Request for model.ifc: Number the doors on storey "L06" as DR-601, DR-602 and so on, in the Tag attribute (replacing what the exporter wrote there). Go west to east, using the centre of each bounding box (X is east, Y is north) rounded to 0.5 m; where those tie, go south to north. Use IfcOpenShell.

First a look at what the model holds.

```python
import ifcopenshell
import ifcopenshell.util.element
import ifcopenshell.util.placement

model = ifcopenshell.open("model.ifc")
print(model.schema)
storey = next(s for s in model.by_type("IfcBuildingStorey") if s.Name == "L06")
doors = [e for e in ifcopenshell.util.element.get_decomposition(storey) if e.is_a("IfcDoor")]
for e in sorted(doors, key=lambda e: e.id()):
    origin = ifcopenshell.util.placement.get_local_placement(e.ObjectPlacement)[:3, 3]
    print(e.id(), e.Tag, e.Name, origin.round(2) + 0.0, sep=" | ")
```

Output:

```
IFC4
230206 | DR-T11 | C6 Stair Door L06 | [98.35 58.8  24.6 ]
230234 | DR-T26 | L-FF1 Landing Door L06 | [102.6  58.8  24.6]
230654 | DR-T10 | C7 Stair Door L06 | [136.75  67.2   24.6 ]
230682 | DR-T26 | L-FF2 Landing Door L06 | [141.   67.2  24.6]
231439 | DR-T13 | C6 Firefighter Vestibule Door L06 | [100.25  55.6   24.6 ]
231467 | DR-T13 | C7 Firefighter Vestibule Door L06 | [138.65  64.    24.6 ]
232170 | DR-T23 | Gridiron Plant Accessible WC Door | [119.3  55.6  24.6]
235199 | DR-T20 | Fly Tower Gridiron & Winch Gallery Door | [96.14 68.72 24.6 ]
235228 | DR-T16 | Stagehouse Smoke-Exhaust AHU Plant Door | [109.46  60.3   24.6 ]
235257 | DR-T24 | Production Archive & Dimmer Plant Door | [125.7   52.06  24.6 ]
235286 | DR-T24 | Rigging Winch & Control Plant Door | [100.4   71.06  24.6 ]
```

```python
import ifcopenshell
import ifcopenshell.geom
import ifcopenshell.util.element
import ifcopenshell.util.shape

model = ifcopenshell.open("model.ifc")
settings = ifcopenshell.geom.settings()
settings.set("use-world-coords", True)


def centre(element):
    shape = ifcopenshell.geom.create_shape(settings, element)
    return ifcopenshell.util.shape.get_bbox_centroid(shape.geometry)


storey = next(s for s in model.by_type("IfcBuildingStorey") if s.Name == "L06")
doors = [e for e in ifcopenshell.util.element.get_decomposition(storey) if e.is_a("IfcDoor")]

# Insertion points can sit at a corner or the storey origin, so sort by the geometry (in metres).
centres = {e: centre(e) for e in doors}
doors.sort(key=lambda e: (round(centres[e][0] / 0.5), centres[e][1]))

for i, e in enumerate(doors, start=1):
    number = f"DR-6{i:02d}"
    e.Tag = number
    print(e.id(), number)

model.write("model_v2.ifc")
```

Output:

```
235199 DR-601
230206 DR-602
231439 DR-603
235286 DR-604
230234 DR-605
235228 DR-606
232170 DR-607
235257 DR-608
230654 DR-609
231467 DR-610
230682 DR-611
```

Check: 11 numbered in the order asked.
